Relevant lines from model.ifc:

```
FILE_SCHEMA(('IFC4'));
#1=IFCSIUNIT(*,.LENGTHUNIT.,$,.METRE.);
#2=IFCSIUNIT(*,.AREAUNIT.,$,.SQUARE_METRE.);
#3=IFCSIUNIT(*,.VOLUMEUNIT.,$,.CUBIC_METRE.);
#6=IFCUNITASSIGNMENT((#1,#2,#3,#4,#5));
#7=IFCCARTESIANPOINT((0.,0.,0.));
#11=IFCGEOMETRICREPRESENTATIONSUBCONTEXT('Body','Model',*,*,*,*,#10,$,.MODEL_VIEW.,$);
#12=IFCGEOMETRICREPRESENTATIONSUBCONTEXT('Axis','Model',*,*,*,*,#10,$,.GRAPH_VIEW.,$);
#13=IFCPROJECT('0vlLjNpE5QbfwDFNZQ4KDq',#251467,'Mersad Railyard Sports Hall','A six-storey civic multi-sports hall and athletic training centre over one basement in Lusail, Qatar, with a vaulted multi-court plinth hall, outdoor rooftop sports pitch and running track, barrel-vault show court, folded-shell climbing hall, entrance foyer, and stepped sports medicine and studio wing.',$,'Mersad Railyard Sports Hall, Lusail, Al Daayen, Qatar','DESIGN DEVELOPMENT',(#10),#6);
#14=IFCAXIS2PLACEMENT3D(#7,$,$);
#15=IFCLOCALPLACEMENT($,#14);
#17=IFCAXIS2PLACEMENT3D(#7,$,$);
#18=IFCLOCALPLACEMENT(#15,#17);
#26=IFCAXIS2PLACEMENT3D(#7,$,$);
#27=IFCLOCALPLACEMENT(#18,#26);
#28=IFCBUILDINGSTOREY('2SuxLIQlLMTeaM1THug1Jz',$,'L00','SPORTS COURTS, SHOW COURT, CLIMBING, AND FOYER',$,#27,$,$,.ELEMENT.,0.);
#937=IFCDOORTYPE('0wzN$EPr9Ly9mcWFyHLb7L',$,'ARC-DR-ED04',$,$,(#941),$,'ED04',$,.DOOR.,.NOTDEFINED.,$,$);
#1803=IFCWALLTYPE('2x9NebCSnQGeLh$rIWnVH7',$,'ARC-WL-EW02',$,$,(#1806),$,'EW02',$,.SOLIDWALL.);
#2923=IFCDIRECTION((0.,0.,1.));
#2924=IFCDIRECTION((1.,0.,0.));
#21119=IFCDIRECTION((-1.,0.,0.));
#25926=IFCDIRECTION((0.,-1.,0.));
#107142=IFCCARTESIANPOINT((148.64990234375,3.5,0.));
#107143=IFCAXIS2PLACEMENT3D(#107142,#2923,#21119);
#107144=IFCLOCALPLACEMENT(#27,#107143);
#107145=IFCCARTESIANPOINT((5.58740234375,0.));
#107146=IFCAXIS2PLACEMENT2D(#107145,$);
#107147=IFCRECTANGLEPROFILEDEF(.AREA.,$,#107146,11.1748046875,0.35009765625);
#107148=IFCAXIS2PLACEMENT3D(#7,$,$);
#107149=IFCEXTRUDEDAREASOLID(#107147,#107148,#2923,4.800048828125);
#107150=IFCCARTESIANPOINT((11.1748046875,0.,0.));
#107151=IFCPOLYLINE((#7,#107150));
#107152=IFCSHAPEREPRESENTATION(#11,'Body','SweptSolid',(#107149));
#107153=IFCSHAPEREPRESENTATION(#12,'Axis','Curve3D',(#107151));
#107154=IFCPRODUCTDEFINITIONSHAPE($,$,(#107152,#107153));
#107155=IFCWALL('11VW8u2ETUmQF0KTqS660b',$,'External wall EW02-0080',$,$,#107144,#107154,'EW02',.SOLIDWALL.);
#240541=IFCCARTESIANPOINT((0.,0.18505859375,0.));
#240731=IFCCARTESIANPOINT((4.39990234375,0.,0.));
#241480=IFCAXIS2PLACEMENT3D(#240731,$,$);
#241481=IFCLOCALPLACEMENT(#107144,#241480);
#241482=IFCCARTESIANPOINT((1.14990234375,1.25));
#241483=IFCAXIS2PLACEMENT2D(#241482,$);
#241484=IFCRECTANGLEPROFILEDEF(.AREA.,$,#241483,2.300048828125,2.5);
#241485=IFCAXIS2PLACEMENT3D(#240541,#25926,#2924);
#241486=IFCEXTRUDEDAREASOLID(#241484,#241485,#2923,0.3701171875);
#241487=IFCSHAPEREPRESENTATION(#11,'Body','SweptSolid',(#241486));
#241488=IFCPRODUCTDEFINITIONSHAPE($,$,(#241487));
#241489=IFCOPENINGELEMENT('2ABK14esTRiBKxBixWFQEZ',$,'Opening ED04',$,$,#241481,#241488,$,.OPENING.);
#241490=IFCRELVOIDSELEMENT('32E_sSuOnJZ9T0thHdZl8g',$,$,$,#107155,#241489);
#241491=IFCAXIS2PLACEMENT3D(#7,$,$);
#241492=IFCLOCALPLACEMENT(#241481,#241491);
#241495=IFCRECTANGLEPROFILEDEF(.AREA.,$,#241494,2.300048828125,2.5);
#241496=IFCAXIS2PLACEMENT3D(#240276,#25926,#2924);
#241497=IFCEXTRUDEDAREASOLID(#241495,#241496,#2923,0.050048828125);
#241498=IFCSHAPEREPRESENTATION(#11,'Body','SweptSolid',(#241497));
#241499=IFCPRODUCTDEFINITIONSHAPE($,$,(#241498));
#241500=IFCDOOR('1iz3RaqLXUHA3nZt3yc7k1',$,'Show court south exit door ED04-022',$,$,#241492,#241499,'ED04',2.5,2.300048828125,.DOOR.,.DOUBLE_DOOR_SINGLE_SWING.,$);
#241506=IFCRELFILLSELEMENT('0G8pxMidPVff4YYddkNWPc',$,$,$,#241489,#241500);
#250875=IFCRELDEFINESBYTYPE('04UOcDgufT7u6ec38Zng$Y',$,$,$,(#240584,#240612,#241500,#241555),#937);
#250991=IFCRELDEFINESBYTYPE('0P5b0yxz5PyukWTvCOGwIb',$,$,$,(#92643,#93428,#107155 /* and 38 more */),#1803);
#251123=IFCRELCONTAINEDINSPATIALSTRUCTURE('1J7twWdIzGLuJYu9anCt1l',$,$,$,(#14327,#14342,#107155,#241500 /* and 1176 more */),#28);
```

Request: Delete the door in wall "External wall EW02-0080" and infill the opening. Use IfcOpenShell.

```python
import ifcopenshell
import ifcopenshell.api.feature
import ifcopenshell.api.root
import ifcopenshell.geom
import ifcopenshell.util.shape

model = ifcopenshell.open("model.ifc")
settings = ifcopenshell.geom.settings()


def volume(element):
    """Net volume in cubic metres, openings subtracted."""
    shape = ifcopenshell.geom.create_shape(settings, element)
    return ifcopenshell.util.shape.get_volume(shape.geometry)


door = model.by_id(241500)
opening = door.FillsVoids[0].RelatingOpeningElement
wall = opening.VoidsElements[0].RelatingBuildingElement
before = volume(wall)

ifcopenshell.api.root.remove_product(model, product=door)
ifcopenshell.api.feature.remove_feature(model, feature=opening)

after = volume(wall)

print(f"wall volume {before:.3f} -> {after:.3f} m3")

model.write("model_edited.ifc")
```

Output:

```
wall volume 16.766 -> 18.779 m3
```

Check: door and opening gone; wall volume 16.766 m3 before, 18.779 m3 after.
